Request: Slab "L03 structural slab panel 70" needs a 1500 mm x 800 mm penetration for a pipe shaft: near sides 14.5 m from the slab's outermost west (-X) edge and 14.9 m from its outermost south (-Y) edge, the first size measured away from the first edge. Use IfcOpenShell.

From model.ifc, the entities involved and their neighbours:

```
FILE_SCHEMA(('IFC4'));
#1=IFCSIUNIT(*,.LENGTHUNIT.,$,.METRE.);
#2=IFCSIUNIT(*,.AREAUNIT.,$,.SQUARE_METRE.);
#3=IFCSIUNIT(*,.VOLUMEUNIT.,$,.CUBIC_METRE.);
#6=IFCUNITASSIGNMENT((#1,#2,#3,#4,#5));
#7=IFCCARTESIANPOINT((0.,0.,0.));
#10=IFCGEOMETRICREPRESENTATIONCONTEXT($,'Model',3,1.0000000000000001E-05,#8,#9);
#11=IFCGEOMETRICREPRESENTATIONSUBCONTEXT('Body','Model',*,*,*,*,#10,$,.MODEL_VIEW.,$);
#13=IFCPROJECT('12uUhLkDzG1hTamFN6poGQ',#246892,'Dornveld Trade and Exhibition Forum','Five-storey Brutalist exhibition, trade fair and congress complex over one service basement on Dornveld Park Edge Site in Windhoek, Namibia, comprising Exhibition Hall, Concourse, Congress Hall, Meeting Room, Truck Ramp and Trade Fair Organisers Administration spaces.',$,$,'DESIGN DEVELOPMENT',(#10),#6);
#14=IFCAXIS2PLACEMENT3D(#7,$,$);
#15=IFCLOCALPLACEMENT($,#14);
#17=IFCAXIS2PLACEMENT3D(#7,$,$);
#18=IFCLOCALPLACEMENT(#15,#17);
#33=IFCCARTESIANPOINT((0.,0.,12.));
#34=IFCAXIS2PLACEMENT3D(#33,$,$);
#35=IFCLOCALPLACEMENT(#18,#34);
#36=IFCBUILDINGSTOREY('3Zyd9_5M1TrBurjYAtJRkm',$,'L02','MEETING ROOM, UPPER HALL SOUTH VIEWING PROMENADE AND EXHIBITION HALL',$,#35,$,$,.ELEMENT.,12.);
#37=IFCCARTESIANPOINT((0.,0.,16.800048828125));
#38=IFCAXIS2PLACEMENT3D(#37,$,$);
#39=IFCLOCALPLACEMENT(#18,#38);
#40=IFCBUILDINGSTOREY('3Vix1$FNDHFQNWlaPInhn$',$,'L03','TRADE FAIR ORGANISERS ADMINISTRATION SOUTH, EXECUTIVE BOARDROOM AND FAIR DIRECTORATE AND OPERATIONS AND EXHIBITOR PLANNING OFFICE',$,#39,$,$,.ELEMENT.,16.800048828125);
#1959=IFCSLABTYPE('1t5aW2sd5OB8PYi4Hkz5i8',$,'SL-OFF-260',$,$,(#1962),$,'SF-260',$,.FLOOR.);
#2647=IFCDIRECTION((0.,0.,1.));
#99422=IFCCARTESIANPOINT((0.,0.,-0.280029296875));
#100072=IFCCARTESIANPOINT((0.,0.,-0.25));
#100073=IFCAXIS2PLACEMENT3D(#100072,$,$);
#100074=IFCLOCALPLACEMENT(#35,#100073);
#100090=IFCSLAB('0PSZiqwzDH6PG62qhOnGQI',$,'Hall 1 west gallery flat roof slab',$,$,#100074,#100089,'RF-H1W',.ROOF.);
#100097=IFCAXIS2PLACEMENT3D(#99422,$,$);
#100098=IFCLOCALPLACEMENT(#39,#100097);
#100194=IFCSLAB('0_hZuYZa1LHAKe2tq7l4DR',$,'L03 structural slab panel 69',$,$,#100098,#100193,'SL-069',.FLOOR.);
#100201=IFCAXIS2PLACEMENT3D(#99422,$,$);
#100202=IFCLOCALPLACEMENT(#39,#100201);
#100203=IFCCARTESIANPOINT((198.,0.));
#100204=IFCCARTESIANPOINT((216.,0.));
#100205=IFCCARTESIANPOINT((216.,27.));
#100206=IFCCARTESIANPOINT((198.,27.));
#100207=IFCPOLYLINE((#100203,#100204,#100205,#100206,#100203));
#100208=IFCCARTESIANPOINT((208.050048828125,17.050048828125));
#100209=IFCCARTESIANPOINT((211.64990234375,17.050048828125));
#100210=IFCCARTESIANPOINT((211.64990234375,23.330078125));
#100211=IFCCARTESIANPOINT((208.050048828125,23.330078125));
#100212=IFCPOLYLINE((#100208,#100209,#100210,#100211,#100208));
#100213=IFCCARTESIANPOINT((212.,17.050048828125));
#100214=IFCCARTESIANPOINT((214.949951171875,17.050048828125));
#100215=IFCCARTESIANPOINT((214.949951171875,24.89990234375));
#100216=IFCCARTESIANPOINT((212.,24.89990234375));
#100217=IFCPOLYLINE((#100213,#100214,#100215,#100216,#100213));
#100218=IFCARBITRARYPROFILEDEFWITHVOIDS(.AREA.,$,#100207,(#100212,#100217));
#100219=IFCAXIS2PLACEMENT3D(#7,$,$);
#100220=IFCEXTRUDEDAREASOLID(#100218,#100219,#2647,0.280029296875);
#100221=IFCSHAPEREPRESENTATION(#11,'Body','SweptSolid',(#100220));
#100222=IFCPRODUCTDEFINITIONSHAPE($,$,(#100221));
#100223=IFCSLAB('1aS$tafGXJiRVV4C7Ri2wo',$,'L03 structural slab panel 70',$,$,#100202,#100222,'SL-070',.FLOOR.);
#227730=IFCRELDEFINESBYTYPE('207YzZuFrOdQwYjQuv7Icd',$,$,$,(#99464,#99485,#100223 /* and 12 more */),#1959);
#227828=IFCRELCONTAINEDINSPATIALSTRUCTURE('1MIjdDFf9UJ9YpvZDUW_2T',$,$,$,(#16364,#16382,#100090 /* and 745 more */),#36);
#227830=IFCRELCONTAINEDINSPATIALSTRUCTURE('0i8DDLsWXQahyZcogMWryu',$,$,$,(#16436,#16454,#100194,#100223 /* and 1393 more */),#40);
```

```python
import numpy as np
import ifcopenshell
import ifcopenshell.api.feature
import ifcopenshell.api.geometry
import ifcopenshell.api.root
import ifcopenshell.geom
import ifcopenshell.util.placement
import ifcopenshell.util.representation
import ifcopenshell.util.shape
import ifcopenshell.util.unit

model = ifcopenshell.open("model.ifc")
unit_scale = ifcopenshell.util.unit.calculate_unit_scale(model)
settings = ifcopenshell.geom.settings()


def volume(element):
    """Net volume in cubic metres, openings subtracted."""
    shape = ifcopenshell.geom.create_shape(settings, element)
    return ifcopenshell.util.shape.get_volume(shape.geometry)


slab = model.by_id(100223)
before = volume(slab)

# Extent in the slab's own axes, in metres. The edges named are its -X and -Y sides.
slab_shape = ifcopenshell.geom.create_shape(settings, slab)
vertices = ifcopenshell.util.shape.get_vertices(slab_shape.geometry)
x_min, y_min, bottom = vertices.min(axis=0)
top = vertices[:, 2].max()

opening = ifcopenshell.api.root.create_entity(model, ifc_class="IfcOpeningElement", name="Pipe shaft opening", predefined_type="OPENING")
context = ifcopenshell.util.representation.get_context(model, "Model", "Body", "MODEL_VIEW")
width, depth = 1.5, 0.8
outline = [(0.0, 0.0), (width, 0.0), (width, depth), (0.0, depth), (0.0, 0.0)]
# Overshoot both faces by 50 mm so the cut is clean.
shape = ifcopenshell.api.geometry.add_slab_representation(
    model, context=context, depth=top - bottom + 0.1, polyline=outline
)
ifcopenshell.api.geometry.assign_representation(model, product=opening, representation=shape)

matrix = ifcopenshell.util.placement.get_local_placement(slab.ObjectPlacement)
matrix[:, 3] = matrix @ np.append(np.array([x_min + 14.5, y_min + 14.9, bottom - 0.05]) / unit_scale, 1.0)
ifcopenshell.api.geometry.edit_object_placement(model, product=opening, matrix=matrix, is_si=False)
ifcopenshell.api.feature.add_feature(model, feature=opening, element=slab)

after = volume(slab)

print(f"slab volume {before:.3f} -> {after:.3f} m3")

model.write("model-out.ifc")
```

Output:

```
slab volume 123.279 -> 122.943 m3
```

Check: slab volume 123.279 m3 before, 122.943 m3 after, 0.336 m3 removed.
